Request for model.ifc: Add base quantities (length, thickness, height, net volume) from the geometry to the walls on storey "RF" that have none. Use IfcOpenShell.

First a look at what the model holds.

```python
import ifcopenshell
import ifcopenshell.util.element
import ifcopenshell.util.unit

model = ifcopenshell.open("model.ifc")
print(model.schema)
for unit_type in ("LENGTHUNIT", "AREAUNIT", "VOLUMEUNIT"):
    print(unit_type, ifcopenshell.util.unit.calculate_unit_scale(model, unit_type))
storey = next(s for s in model.by_type("IfcBuildingStorey") if s.Name == "RF")
walls = [e for e in ifcopenshell.util.element.get_decomposition(storey) if e.is_a("IfcWall")]
for e in sorted(walls, key=lambda e: e.id()):
    print(e.id(), e.is_a(), e.Name, list(ifcopenshell.util.element.get_psets(e, qtos_only=True)), sep=" | ")
```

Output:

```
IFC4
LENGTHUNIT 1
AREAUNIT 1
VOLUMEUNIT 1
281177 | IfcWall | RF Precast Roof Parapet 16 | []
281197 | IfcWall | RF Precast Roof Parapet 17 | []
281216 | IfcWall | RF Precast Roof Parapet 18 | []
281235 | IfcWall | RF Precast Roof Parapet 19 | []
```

```python
import ifcopenshell
import ifcopenshell.api.pset
import ifcopenshell.geom
import ifcopenshell.util.element
import ifcopenshell.util.shape
import ifcopenshell.util.unit

model = ifcopenshell.open("model.ifc")
unit_scale = ifcopenshell.util.unit.calculate_unit_scale(model)
volume_scale = ifcopenshell.util.unit.calculate_unit_scale(model, "VOLUMEUNIT")
settings = ifcopenshell.geom.settings()

storey = next(s for s in model.by_type("IfcBuildingStorey") if s.Name == "RF")
walls = [e for e in ifcopenshell.util.element.get_decomposition(storey) if e.is_a("IfcWall")]

for e in sorted(walls, key=lambda e: e.id()):
    if ifcopenshell.util.element.get_psets(e, qtos_only=True, should_inherit=False):
        continue
    # Geometry comes back in metres, in the element's own axes.
    shape = ifcopenshell.geom.create_shape(settings, e)
    values = {
        "Length": ifcopenshell.util.shape.get_x(shape.geometry) / unit_scale,
        "Width": ifcopenshell.util.shape.get_y(shape.geometry) / unit_scale,
        "Height": ifcopenshell.util.shape.get_z(shape.geometry) / unit_scale,
        "NetVolume": ifcopenshell.util.shape.get_volume(shape.geometry) / volume_scale,
    }
    qto = ifcopenshell.api.pset.add_qto(model, product=e, name="Qto_WallBaseQuantities")
    ifcopenshell.api.pset.edit_qto(model, qto=qto, properties=values)
    print(e.id(), {k: round(v, 3) for k, v in values.items()})

model.write("model_updated.ifc")
```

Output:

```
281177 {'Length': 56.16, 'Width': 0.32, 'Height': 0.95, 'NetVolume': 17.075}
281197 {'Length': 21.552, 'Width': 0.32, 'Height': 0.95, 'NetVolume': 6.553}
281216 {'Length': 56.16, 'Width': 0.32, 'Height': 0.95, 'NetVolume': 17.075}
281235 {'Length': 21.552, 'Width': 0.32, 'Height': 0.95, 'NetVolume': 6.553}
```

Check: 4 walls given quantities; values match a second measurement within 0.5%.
